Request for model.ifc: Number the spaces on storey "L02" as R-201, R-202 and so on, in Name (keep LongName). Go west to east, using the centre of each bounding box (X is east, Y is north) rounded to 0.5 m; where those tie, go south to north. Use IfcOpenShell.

First a look at what the model holds.

```python
import ifcopenshell
import ifcopenshell.util.element
import ifcopenshell.util.placement

model = ifcopenshell.open("model.ifc")
print(model.schema)
storey = next(s for s in model.by_type("IfcBuildingStorey") if s.Name == "L02")
spaces = [e for e in ifcopenshell.util.element.get_decomposition(storey) if e.is_a("IfcSpace")]
for e in sorted(spaces, key=lambda e: e.id()):
    origin = ifcopenshell.util.placement.get_local_placement(e.ObjectPlacement)[:3, 3]
    print(e.id(), e.Name, e.LongName, origin.round(2) + 0.0, sep=" | ")
```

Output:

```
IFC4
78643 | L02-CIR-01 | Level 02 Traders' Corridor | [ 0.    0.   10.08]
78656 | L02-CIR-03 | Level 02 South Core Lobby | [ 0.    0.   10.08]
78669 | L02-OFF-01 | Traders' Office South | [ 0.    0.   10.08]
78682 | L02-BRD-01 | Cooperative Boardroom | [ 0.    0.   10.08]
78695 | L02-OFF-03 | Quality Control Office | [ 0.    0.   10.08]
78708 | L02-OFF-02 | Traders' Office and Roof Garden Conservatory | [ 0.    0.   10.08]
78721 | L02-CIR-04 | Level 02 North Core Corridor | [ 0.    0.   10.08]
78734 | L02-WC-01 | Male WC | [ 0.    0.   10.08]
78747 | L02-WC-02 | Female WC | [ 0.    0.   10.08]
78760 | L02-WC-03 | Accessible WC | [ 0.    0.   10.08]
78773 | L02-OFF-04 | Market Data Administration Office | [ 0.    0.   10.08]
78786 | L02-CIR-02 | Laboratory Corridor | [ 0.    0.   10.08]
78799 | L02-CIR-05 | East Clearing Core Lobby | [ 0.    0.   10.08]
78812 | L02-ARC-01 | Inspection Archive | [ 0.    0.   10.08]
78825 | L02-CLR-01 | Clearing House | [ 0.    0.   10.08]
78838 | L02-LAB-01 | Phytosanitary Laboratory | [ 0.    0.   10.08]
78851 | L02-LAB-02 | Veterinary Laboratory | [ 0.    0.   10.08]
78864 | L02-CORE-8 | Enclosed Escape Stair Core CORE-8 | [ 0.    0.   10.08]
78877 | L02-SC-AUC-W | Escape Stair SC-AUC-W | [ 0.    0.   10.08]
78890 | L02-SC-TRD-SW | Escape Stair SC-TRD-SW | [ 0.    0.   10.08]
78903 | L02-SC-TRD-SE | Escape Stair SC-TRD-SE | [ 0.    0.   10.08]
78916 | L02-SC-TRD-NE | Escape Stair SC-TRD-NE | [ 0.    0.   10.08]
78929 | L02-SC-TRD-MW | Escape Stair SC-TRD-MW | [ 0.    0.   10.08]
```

```python
import ifcopenshell
import ifcopenshell.geom
import ifcopenshell.util.element
import ifcopenshell.util.shape

model = ifcopenshell.open("model.ifc")
settings = ifcopenshell.geom.settings()
settings.set("use-world-coords", True)


def centre(element):
    shape = ifcopenshell.geom.create_shape(settings, element)
    return ifcopenshell.util.shape.get_bbox_centroid(shape.geometry)


storey = next(s for s in model.by_type("IfcBuildingStorey") if s.Name == "L02")
spaces = [e for e in ifcopenshell.util.element.get_decomposition(storey) if e.is_a("IfcSpace")]

# Insertion points can sit at a corner or the storey origin, so sort by the geometry (in metres).
centres = {e: centre(e) for e in spaces}
spaces.sort(key=lambda e: (round(centres[e][0] / 0.5), centres[e][1]))

for i, e in enumerate(spaces, start=1):
    number = f"R-2{i:02d}"
    e.Name = number
    print(e.id(), number)

model.write("model_edited.ifc")
```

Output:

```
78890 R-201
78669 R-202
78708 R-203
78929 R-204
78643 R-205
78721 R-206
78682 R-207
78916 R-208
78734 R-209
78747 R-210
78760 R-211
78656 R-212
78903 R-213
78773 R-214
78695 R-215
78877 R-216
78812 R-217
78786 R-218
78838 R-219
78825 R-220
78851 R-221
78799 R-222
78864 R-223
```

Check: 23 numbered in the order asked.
